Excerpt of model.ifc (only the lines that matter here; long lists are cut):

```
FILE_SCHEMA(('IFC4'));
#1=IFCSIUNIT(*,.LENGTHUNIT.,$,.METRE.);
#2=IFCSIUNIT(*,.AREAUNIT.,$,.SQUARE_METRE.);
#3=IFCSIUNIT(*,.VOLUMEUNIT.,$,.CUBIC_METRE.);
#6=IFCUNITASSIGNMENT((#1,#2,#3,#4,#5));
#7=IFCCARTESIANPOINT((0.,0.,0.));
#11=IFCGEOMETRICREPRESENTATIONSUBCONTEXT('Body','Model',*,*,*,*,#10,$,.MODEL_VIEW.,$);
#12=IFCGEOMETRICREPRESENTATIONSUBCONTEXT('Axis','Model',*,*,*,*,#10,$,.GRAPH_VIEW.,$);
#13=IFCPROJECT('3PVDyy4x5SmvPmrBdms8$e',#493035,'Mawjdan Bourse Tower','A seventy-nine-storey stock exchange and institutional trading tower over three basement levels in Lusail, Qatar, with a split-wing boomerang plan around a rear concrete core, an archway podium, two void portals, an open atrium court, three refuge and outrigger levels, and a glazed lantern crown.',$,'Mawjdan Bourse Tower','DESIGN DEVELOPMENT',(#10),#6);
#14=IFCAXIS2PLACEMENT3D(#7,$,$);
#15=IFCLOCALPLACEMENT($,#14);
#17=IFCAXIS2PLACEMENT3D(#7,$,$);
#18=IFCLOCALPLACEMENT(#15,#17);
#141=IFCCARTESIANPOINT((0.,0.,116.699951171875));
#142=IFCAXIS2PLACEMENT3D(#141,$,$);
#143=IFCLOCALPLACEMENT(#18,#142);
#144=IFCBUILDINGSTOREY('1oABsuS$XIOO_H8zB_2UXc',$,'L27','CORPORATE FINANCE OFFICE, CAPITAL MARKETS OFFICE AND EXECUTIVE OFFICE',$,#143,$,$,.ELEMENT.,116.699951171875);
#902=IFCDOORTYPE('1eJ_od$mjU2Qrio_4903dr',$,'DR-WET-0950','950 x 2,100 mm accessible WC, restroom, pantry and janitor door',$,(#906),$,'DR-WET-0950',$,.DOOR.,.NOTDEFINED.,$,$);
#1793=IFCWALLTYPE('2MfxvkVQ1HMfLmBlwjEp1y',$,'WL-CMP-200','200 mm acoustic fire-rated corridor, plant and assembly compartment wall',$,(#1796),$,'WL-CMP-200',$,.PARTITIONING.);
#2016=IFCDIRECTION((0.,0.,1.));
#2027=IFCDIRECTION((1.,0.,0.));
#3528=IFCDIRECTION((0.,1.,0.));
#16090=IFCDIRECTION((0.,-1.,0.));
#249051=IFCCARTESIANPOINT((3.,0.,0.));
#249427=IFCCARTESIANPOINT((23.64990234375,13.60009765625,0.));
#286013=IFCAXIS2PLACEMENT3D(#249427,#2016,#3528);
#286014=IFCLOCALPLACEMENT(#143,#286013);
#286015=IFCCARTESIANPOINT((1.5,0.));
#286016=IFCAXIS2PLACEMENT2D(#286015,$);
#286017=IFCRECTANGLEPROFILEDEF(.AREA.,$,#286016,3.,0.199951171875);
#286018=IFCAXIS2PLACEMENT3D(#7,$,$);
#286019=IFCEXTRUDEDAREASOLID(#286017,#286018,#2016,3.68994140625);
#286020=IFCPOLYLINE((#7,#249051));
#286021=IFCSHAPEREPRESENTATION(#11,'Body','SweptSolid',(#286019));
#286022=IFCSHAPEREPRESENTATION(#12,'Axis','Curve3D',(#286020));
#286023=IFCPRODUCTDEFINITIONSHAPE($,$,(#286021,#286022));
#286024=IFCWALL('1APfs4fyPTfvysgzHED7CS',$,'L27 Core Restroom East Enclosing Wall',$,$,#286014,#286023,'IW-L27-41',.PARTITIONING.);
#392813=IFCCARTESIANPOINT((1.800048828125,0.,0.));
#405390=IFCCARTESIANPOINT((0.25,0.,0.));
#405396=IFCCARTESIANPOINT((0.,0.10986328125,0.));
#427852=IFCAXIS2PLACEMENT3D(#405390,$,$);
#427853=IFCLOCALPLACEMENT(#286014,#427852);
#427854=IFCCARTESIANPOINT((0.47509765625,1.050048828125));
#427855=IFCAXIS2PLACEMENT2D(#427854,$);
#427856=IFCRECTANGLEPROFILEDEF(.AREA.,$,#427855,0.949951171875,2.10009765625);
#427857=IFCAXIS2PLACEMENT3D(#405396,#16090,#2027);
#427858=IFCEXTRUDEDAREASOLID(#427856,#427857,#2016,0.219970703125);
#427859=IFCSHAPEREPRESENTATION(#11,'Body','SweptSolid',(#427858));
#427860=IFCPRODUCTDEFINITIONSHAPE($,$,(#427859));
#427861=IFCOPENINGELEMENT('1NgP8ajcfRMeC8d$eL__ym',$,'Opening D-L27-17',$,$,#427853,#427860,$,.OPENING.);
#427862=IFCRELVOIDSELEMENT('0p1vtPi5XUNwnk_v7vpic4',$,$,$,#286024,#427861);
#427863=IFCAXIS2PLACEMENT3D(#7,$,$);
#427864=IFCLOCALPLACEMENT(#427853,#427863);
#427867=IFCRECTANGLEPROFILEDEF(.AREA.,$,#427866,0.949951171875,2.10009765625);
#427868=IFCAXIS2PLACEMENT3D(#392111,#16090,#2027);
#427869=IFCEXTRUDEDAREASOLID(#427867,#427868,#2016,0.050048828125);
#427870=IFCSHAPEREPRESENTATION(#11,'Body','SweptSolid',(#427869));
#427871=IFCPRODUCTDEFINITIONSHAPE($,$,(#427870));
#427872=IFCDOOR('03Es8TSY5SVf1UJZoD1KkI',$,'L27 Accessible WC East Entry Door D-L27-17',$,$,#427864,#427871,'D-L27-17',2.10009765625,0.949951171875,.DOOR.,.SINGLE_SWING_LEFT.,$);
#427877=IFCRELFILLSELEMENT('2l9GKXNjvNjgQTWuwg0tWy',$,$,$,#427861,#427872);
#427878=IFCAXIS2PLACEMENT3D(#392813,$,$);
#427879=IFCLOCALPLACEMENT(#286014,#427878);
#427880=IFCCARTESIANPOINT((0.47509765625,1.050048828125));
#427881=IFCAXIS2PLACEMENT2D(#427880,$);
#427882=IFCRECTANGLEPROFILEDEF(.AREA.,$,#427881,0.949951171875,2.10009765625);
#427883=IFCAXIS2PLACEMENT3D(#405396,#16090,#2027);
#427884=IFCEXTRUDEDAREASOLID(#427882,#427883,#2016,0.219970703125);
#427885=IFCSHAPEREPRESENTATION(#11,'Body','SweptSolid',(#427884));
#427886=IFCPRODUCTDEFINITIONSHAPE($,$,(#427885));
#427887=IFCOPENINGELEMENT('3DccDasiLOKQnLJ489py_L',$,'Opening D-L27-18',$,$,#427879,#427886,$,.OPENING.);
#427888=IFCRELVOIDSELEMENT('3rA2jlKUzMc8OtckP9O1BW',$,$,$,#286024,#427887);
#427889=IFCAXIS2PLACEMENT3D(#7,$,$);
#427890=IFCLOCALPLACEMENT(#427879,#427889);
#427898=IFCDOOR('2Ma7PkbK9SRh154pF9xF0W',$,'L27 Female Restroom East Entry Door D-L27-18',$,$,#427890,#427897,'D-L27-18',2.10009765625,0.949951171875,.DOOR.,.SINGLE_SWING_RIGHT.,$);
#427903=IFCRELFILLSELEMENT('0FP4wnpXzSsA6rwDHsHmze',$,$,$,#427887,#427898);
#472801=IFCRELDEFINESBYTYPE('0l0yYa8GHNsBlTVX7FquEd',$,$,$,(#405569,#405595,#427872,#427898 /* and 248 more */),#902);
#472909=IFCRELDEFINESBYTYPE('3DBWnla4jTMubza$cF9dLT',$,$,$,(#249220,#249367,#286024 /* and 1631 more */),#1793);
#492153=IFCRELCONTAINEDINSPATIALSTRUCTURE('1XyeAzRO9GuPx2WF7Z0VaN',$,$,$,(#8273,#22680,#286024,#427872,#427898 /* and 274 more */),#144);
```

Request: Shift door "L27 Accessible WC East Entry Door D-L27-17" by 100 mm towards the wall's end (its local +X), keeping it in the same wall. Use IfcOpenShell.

```python
import ifcopenshell
import ifcopenshell.api.geometry
import ifcopenshell.util.placement

model = ifcopenshell.open("model.ifc")

door = model.by_guid("03Es8TSY5SVf1UJZoD1KkI")
opening = door.FillsVoids[0].RelatingOpeningElement
wall = opening.VoidsElements[0].RelatingBuildingElement

wall_matrix = ifcopenshell.util.placement.get_local_placement(wall.ObjectPlacement)
shift = wall_matrix[:3, 0] * 0.1
before = ifcopenshell.util.placement.get_local_placement(door.ObjectPlacement)[:3, 3].copy()

# The door is placed relative to its opening, so it follows when the opening moves.
matrix = ifcopenshell.util.placement.get_local_placement(opening.ObjectPlacement)
matrix[:3, 3] += shift
ifcopenshell.api.geometry.edit_object_placement(
    model, product=opening, matrix=matrix, is_si=False, should_transform_children=True
)

after = ifcopenshell.util.placement.get_local_placement(door.ObjectPlacement)[:3, 3]
print("door moved by", (after - before).round(3) + 0.0)

model.write("model_edited.ifc")
```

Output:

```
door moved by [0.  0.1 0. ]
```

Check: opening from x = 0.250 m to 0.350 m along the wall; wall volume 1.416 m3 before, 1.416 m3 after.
